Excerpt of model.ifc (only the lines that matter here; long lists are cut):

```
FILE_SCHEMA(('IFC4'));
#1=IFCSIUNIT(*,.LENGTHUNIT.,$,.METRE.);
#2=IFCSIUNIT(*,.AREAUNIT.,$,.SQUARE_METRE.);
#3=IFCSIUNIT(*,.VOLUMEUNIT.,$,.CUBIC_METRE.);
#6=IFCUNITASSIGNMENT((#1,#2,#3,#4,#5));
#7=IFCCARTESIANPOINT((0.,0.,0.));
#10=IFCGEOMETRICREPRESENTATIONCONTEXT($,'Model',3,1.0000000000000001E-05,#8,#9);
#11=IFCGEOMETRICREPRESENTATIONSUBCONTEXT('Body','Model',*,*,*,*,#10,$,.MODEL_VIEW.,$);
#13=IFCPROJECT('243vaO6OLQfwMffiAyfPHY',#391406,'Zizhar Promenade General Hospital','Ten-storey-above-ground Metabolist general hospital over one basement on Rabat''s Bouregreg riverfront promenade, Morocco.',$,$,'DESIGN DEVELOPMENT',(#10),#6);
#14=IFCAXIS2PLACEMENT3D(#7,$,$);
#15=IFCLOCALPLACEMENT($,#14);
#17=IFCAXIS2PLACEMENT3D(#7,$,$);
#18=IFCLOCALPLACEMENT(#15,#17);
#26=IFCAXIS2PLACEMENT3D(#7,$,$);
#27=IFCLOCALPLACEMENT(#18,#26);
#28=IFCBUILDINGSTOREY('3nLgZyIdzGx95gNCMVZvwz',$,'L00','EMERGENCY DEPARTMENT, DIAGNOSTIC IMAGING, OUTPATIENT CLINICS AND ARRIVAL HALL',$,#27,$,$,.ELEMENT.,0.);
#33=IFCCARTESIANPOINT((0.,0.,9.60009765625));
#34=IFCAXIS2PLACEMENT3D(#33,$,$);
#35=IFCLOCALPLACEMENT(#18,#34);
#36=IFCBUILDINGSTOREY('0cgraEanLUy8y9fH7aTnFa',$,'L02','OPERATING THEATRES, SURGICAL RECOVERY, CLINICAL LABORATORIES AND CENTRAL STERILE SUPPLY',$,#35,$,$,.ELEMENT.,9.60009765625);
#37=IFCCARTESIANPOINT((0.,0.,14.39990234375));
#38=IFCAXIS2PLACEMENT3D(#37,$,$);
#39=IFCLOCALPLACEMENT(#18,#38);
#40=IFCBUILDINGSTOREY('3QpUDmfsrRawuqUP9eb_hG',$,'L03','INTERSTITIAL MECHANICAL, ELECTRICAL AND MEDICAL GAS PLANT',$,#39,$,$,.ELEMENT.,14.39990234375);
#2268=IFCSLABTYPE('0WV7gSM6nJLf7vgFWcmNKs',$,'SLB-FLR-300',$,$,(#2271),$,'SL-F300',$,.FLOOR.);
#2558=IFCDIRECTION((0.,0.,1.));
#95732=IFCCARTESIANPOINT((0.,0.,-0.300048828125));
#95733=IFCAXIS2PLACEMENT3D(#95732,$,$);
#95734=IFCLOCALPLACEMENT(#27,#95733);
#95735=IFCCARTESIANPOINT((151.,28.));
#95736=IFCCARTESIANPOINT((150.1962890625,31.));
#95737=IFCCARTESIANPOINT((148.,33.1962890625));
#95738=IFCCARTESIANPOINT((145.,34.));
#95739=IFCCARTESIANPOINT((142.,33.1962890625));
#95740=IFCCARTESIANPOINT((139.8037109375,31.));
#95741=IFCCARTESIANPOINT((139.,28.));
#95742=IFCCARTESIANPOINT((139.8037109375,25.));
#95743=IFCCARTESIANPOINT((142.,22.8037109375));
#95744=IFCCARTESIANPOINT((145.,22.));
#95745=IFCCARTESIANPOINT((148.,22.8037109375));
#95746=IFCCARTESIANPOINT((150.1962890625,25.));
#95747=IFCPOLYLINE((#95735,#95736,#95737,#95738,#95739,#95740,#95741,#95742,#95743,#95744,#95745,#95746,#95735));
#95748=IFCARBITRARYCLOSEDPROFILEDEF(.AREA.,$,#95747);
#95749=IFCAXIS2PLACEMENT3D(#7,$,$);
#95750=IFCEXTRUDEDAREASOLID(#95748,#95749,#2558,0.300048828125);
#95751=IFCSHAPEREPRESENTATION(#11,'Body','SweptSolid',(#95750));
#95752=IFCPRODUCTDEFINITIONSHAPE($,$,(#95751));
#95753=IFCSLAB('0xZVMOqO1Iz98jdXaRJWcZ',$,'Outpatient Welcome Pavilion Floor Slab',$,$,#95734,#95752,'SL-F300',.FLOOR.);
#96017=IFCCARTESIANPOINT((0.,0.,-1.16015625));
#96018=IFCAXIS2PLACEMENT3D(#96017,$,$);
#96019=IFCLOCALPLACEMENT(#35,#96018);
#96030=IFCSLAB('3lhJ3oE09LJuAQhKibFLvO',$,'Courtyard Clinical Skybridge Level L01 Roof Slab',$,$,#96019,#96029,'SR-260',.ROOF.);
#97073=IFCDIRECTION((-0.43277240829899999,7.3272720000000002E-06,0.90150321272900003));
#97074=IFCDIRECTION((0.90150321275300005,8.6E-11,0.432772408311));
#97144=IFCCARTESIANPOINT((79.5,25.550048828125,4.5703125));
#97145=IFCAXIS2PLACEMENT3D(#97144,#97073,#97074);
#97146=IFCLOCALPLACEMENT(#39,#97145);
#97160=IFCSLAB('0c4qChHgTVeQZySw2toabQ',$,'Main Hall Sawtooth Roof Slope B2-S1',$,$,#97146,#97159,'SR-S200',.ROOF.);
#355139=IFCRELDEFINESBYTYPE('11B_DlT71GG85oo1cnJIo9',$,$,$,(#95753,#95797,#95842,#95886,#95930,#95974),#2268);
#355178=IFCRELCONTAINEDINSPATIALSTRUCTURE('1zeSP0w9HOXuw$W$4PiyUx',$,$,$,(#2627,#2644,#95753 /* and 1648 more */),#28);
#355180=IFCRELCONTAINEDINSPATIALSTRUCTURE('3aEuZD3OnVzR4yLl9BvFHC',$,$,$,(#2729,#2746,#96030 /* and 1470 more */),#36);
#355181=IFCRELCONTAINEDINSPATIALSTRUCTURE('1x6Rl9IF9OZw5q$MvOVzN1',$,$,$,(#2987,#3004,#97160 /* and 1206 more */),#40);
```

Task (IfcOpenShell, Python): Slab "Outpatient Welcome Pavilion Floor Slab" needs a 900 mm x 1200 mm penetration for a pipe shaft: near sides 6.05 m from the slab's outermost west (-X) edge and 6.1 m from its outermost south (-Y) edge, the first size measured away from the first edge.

```python
import numpy as np
import ifcopenshell
import ifcopenshell.api.feature
import ifcopenshell.api.geometry
import ifcopenshell.api.root
import ifcopenshell.geom
import ifcopenshell.util.placement
import ifcopenshell.util.representation
import ifcopenshell.util.shape
import ifcopenshell.util.unit

model = ifcopenshell.open("model.ifc")
unit_scale = ifcopenshell.util.unit.calculate_unit_scale(model)
settings = ifcopenshell.geom.settings()


def volume(element):
    """Net volume in cubic metres, openings subtracted."""
    shape = ifcopenshell.geom.create_shape(settings, element)
    return ifcopenshell.util.shape.get_volume(shape.geometry)


slab = model.by_id(95753)
before = volume(slab)

# Extent in the slab's own axes, in metres. The edges named are its -X and -Y sides.
slab_shape = ifcopenshell.geom.create_shape(settings, slab)
vertices = ifcopenshell.util.shape.get_vertices(slab_shape.geometry)
x_min, y_min, bottom = vertices.min(axis=0)
top = vertices[:, 2].max()

opening = ifcopenshell.api.root.create_entity(model, ifc_class="IfcOpeningElement", name="Pipe shaft opening", predefined_type="OPENING")
context = ifcopenshell.util.representation.get_context(model, "Model", "Body", "MODEL_VIEW")
width, depth = 0.9, 1.2
outline = [(0.0, 0.0), (width, 0.0), (width, depth), (0.0, depth), (0.0, 0.0)]
# Overshoot both faces by 50 mm so the cut is clean.
shape = ifcopenshell.api.geometry.add_slab_representation(
    model, context=context, depth=top - bottom + 0.1, polyline=outline
)
ifcopenshell.api.geometry.assign_representation(model, product=opening, representation=shape)

matrix = ifcopenshell.util.placement.get_local_placement(slab.ObjectPlacement)
matrix[:, 3] = matrix @ np.append(np.array([x_min + 6.05, y_min + 6.1, bottom - 0.05]) / unit_scale, 1.0)
ifcopenshell.api.geometry.edit_object_placement(model, product=opening, matrix=matrix, is_si=False)
ifcopenshell.api.feature.add_feature(model, feature=opening, element=slab)

after = volume(slab)

print(f"slab volume {before:.3f} -> {after:.3f} m3")

model.write("model_v2.ifc")
```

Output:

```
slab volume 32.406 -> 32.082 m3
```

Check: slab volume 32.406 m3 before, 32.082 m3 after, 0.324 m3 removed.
